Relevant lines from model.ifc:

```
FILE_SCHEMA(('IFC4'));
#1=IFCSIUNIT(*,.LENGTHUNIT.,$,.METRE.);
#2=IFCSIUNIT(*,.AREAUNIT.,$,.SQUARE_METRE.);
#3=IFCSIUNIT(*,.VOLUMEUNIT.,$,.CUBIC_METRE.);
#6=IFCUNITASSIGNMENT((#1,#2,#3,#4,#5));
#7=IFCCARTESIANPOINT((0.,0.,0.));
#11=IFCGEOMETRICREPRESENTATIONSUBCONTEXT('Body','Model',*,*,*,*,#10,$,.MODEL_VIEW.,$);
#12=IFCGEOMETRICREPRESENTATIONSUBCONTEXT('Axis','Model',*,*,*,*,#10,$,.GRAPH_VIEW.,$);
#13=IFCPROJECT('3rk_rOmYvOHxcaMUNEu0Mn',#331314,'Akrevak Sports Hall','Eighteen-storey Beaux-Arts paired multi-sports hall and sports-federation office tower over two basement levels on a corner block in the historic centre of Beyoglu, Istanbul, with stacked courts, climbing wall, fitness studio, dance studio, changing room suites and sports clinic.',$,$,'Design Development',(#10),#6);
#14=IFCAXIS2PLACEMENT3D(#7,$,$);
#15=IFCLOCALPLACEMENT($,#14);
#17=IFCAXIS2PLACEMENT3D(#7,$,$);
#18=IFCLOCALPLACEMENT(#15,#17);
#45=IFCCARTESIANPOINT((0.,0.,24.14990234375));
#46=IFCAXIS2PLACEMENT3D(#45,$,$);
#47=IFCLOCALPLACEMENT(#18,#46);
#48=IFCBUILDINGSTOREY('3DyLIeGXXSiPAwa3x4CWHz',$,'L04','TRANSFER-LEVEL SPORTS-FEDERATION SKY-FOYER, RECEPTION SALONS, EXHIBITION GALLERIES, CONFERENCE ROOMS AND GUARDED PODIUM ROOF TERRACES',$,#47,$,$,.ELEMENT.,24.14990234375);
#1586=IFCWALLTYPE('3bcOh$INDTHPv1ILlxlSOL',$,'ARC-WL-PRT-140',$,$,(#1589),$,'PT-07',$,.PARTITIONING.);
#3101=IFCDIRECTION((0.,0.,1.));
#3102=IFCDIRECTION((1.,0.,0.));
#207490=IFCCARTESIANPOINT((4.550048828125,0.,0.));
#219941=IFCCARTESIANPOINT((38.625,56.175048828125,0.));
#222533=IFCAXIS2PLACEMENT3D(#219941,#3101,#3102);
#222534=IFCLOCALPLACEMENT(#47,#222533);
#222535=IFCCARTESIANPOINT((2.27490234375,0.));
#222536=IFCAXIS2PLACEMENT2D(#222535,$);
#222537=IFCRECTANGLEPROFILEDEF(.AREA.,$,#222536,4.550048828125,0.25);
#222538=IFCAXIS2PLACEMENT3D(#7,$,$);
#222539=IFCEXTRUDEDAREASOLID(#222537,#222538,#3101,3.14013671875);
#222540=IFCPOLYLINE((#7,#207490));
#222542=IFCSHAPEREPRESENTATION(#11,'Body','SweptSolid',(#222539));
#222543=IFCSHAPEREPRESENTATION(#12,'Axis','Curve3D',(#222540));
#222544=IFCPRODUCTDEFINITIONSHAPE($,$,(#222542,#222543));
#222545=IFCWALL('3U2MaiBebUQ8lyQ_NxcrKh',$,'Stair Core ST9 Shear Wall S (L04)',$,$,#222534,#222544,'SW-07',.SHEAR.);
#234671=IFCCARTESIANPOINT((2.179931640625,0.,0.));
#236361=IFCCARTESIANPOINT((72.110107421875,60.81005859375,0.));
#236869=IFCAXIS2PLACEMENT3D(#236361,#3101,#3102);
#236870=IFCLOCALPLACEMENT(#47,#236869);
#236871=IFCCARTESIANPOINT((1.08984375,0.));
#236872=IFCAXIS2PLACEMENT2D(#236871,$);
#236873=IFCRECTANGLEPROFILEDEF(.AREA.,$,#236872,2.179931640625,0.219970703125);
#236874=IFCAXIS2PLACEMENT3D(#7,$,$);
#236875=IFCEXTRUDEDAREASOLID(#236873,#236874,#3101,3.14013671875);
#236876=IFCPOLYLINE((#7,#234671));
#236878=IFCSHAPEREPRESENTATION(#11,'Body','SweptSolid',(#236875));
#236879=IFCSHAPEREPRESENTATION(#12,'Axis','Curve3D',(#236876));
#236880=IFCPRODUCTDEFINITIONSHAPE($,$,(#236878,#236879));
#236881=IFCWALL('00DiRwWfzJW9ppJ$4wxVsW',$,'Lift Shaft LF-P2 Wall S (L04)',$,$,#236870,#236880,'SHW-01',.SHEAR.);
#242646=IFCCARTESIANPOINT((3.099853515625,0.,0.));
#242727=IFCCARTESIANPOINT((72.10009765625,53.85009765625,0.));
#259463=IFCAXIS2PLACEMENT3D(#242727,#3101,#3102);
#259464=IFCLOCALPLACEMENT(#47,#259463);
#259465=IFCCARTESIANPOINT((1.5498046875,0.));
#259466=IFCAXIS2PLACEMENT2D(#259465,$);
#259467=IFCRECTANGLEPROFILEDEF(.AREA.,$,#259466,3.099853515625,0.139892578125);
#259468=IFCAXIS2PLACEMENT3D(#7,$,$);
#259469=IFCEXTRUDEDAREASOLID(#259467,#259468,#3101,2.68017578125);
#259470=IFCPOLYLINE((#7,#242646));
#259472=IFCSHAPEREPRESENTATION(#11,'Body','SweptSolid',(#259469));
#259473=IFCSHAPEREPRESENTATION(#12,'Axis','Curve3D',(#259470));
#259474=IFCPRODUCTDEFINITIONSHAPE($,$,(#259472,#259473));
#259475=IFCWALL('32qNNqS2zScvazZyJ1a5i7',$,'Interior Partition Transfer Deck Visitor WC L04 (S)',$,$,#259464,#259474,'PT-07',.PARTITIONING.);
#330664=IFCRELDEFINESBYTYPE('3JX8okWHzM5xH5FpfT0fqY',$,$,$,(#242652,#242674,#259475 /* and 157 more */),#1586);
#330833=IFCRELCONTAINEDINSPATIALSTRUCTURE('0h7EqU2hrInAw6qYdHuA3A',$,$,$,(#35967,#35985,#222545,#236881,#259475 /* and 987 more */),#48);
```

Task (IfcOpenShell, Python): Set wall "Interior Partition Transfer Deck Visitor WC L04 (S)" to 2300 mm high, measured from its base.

```python
import ifcopenshell
import ifcopenshell.geom
import ifcopenshell.util.representation
import ifcopenshell.util.shape

model = ifcopenshell.open("model.ifc")
settings = ifcopenshell.geom.settings()


def volume(element):
    """Net volume in cubic metres, openings subtracted."""
    shape = ifcopenshell.geom.create_shape(settings, element)
    return ifcopenshell.util.shape.get_volume(shape.geometry)


wall = model.by_id(259475)
before = volume(wall)

body = ifcopenshell.util.representation.get_representation(wall, "Model", "Body")
solid = body.Items[0]
old_height = solid.Depth
solid.Depth = 2.3
after = volume(wall)

print(f"height {old_height:g} -> {solid.Depth:g}, volume {before:.3f} -> {after:.3f} m3")

model.write("model-out.ifc")
```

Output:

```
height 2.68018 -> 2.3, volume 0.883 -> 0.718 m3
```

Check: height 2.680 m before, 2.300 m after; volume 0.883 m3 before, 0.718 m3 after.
